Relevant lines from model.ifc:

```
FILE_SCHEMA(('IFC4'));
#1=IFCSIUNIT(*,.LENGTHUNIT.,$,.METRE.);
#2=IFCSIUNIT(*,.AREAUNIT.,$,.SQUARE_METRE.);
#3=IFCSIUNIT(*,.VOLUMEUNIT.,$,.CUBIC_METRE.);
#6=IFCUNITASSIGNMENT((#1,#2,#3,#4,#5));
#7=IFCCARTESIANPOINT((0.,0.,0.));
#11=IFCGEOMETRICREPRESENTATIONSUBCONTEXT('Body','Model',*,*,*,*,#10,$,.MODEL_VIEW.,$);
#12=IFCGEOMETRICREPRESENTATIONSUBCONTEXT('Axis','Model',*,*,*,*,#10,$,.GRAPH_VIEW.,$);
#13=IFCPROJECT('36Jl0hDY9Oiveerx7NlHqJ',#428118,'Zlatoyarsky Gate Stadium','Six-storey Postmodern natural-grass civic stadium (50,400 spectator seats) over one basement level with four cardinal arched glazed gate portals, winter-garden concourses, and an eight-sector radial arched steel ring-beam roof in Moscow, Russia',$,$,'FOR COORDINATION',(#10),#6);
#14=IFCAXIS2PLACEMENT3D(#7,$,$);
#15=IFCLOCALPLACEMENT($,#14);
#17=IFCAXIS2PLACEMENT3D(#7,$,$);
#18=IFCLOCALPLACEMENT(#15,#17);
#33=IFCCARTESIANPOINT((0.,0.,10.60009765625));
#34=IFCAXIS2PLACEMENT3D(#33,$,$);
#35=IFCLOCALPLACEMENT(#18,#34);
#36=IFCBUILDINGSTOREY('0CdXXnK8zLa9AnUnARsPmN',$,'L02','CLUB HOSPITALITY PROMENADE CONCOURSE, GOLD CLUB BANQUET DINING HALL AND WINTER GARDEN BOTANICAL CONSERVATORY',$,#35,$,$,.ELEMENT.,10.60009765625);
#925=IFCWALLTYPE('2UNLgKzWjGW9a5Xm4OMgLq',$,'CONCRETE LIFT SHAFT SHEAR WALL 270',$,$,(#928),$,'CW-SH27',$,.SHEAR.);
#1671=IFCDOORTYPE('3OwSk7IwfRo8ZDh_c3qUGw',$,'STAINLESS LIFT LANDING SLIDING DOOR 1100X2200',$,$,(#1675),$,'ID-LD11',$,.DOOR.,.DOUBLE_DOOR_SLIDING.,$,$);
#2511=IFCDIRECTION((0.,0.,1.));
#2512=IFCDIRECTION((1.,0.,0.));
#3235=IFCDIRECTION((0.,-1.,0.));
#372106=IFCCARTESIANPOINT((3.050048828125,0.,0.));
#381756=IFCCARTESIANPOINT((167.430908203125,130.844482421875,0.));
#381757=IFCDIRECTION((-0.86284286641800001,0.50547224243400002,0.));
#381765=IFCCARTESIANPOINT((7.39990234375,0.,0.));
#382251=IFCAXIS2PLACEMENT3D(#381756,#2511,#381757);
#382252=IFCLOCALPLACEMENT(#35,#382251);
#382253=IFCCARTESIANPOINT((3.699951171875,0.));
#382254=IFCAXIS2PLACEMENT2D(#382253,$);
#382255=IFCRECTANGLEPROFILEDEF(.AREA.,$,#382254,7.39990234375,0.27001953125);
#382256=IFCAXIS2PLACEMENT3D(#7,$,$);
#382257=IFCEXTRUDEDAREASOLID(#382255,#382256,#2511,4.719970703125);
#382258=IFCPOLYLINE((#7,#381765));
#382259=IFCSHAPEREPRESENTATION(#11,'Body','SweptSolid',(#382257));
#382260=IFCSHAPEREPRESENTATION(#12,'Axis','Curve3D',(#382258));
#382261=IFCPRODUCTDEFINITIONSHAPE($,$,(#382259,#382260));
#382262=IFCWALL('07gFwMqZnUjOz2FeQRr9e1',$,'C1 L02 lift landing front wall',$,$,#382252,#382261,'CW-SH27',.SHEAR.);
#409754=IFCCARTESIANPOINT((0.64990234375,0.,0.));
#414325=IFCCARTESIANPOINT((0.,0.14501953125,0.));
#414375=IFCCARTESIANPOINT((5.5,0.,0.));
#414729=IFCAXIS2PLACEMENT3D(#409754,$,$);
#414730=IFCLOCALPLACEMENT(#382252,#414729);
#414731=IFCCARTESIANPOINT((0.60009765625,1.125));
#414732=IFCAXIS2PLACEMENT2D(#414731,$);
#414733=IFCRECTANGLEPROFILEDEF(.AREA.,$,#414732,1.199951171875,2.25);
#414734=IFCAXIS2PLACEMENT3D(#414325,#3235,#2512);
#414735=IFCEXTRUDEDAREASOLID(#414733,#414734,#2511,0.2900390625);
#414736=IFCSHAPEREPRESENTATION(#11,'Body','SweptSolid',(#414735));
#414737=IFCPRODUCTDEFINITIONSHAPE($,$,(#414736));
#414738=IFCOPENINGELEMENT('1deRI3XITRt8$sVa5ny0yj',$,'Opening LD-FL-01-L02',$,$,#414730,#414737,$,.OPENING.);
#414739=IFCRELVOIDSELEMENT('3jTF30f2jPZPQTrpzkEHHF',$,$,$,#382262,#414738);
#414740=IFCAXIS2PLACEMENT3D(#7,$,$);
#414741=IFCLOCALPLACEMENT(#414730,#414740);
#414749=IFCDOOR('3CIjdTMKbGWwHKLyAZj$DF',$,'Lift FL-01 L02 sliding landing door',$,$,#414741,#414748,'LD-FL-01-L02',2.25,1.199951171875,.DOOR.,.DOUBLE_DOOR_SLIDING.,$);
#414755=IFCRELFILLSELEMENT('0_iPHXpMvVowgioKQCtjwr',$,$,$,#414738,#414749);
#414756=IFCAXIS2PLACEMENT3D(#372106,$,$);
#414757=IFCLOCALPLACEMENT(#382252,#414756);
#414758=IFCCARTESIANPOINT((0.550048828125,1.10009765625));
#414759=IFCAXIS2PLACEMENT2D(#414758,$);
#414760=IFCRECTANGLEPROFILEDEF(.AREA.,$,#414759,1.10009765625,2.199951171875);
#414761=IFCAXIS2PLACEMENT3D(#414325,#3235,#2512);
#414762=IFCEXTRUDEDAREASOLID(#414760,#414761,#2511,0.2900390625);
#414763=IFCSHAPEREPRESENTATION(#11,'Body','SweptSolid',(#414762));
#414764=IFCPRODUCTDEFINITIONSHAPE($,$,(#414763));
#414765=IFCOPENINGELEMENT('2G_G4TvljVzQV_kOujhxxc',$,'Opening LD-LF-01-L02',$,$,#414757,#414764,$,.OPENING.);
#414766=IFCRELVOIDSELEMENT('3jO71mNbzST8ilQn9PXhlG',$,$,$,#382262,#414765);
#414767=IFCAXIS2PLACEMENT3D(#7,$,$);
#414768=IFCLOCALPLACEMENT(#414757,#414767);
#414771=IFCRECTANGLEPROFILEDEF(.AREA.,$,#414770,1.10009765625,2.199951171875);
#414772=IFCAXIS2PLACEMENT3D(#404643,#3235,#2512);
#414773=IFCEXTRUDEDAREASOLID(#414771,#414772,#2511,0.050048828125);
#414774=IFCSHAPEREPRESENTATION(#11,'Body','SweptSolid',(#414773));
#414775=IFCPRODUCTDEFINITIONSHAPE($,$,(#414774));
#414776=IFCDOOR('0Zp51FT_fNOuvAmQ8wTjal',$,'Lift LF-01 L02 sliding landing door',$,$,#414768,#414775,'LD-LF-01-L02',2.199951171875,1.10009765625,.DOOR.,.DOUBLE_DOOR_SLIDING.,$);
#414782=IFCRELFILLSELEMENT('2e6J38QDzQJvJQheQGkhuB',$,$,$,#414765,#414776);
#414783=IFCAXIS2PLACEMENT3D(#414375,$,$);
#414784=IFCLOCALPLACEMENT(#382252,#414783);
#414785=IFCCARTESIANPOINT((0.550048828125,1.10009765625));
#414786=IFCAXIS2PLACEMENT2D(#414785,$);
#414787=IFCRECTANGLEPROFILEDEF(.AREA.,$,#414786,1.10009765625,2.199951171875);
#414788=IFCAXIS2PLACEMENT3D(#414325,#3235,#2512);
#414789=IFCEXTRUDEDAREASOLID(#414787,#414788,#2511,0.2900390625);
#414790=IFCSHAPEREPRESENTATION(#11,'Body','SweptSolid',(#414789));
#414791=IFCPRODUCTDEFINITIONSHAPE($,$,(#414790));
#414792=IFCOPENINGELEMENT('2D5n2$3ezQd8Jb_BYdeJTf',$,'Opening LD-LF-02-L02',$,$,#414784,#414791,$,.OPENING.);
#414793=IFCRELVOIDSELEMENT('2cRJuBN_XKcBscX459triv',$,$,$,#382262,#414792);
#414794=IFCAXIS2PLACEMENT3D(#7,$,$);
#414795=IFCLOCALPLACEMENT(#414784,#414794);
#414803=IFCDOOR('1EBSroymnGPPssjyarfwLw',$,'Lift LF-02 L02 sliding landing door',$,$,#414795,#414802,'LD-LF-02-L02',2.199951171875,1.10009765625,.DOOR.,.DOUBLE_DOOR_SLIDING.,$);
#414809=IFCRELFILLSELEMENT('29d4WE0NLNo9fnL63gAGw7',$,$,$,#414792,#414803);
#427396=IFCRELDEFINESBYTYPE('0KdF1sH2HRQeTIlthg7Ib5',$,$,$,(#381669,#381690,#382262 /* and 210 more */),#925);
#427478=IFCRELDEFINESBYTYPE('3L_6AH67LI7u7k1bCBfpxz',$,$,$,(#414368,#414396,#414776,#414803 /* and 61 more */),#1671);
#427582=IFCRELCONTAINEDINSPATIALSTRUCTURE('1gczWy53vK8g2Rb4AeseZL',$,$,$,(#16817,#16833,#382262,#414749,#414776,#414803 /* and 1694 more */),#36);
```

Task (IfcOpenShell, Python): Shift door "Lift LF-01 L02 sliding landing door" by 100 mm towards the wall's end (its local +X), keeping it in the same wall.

```python
import ifcopenshell
import ifcopenshell.api.geometry
import ifcopenshell.util.placement
import ifcopenshell.util.unit

model = ifcopenshell.open("model.ifc")
unit_scale = ifcopenshell.util.unit.calculate_unit_scale(model)

door = model.by_id(414776)
opening = door.FillsVoids[0].RelatingOpeningElement
wall = opening.VoidsElements[0].RelatingBuildingElement

wall_matrix = ifcopenshell.util.placement.get_local_placement(wall.ObjectPlacement)
shift = wall_matrix[:3, 0] * 0.1 / unit_scale
before = ifcopenshell.util.placement.get_local_placement(door.ObjectPlacement)[:3, 3].copy()

# The door is placed relative to its opening, so it follows when the opening moves.
matrix = ifcopenshell.util.placement.get_local_placement(opening.ObjectPlacement)
matrix[:3, 3] += shift
ifcopenshell.api.geometry.edit_object_placement(
    model, product=opening, matrix=matrix, is_si=False, should_transform_children=True
)

after = ifcopenshell.util.placement.get_local_placement(door.ObjectPlacement)[:3, 3]
print("door moved by", (after - before).round(3) + 0.0)

model.write("model_rev.ifc")
```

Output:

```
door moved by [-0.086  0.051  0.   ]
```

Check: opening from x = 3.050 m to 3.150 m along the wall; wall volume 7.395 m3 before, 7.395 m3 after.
